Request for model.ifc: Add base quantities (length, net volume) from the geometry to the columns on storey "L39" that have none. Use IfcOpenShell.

First a look at what the model holds.

```python
import ifcopenshell
import ifcopenshell.util.element
import ifcopenshell.util.unit

model = ifcopenshell.open("model.ifc")
print(model.schema)
for unit_type in ("LENGTHUNIT", "AREAUNIT", "VOLUMEUNIT"):
    print(unit_type, ifcopenshell.util.unit.calculate_unit_scale(model, unit_type))
storey = next(s for s in model.by_type("IfcBuildingStorey") if s.Name == "L39")
columns = [e for e in ifcopenshell.util.element.get_decomposition(storey) if e.is_a("IfcColumn")]
for e in sorted(columns, key=lambda e: e.id()):
    print(e.id(), e.is_a(), e.Name, list(ifcopenshell.util.element.get_psets(e, qtos_only=True)), sep=" | ")
```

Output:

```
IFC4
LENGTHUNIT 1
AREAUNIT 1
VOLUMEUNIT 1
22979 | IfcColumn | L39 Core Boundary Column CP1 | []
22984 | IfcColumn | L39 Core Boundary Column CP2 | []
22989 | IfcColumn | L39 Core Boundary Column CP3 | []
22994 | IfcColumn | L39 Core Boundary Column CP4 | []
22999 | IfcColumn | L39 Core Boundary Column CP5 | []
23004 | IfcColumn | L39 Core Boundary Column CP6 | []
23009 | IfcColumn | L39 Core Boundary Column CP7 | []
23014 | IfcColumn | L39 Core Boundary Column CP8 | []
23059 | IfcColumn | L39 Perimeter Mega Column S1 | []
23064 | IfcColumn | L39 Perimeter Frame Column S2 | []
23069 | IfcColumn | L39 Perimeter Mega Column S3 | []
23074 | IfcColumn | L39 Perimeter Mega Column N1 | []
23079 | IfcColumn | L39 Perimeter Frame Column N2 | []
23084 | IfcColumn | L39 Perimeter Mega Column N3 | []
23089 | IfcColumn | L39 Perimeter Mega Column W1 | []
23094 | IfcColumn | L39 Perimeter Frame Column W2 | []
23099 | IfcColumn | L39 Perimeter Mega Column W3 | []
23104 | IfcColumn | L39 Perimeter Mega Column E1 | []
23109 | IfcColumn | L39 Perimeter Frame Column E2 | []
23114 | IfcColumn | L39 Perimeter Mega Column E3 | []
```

```python
import ifcopenshell
import ifcopenshell.api.pset
import ifcopenshell.geom
import ifcopenshell.util.element
import ifcopenshell.util.shape
import ifcopenshell.util.unit

model = ifcopenshell.open("model.ifc")
unit_scale = ifcopenshell.util.unit.calculate_unit_scale(model)
volume_scale = ifcopenshell.util.unit.calculate_unit_scale(model, "VOLUMEUNIT")
settings = ifcopenshell.geom.settings()

storey = next(s for s in model.by_type("IfcBuildingStorey") if s.Name == "L39")
columns = [e for e in ifcopenshell.util.element.get_decomposition(storey) if e.is_a("IfcColumn")]

for e in sorted(columns, key=lambda e: e.id()):
    if ifcopenshell.util.element.get_psets(e, qtos_only=True, should_inherit=False):
        continue
    # Geometry comes back in metres, in the element's own axes.
    shape = ifcopenshell.geom.create_shape(settings, e)
    values = {
        "Length": ifcopenshell.util.shape.get_z(shape.geometry) / unit_scale,
        "NetVolume": ifcopenshell.util.shape.get_volume(shape.geometry) / volume_scale,
    }
    qto = ifcopenshell.api.pset.add_qto(model, product=e, name="Qto_ColumnBaseQuantities")
    ifcopenshell.api.pset.edit_qto(model, qto=qto, properties=values)
    print(e.id(), {k: round(v, 3) for k, v in values.items()})

model.write("model_updated.ifc")
```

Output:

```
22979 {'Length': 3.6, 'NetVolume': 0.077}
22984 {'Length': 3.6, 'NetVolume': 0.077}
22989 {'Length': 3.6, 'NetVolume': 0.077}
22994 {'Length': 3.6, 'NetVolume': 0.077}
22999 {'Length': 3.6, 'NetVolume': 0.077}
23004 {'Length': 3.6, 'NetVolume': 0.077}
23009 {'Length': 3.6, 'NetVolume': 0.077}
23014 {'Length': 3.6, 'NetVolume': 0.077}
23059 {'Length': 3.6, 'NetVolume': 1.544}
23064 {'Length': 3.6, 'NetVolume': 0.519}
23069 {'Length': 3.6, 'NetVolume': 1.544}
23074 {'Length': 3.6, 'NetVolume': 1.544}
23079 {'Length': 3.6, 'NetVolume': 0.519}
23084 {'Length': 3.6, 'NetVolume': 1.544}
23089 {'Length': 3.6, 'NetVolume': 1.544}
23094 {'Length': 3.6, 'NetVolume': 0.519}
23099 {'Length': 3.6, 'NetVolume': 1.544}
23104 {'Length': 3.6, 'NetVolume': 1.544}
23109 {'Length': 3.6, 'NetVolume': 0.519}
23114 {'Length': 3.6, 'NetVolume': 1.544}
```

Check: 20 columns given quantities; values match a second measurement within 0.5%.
